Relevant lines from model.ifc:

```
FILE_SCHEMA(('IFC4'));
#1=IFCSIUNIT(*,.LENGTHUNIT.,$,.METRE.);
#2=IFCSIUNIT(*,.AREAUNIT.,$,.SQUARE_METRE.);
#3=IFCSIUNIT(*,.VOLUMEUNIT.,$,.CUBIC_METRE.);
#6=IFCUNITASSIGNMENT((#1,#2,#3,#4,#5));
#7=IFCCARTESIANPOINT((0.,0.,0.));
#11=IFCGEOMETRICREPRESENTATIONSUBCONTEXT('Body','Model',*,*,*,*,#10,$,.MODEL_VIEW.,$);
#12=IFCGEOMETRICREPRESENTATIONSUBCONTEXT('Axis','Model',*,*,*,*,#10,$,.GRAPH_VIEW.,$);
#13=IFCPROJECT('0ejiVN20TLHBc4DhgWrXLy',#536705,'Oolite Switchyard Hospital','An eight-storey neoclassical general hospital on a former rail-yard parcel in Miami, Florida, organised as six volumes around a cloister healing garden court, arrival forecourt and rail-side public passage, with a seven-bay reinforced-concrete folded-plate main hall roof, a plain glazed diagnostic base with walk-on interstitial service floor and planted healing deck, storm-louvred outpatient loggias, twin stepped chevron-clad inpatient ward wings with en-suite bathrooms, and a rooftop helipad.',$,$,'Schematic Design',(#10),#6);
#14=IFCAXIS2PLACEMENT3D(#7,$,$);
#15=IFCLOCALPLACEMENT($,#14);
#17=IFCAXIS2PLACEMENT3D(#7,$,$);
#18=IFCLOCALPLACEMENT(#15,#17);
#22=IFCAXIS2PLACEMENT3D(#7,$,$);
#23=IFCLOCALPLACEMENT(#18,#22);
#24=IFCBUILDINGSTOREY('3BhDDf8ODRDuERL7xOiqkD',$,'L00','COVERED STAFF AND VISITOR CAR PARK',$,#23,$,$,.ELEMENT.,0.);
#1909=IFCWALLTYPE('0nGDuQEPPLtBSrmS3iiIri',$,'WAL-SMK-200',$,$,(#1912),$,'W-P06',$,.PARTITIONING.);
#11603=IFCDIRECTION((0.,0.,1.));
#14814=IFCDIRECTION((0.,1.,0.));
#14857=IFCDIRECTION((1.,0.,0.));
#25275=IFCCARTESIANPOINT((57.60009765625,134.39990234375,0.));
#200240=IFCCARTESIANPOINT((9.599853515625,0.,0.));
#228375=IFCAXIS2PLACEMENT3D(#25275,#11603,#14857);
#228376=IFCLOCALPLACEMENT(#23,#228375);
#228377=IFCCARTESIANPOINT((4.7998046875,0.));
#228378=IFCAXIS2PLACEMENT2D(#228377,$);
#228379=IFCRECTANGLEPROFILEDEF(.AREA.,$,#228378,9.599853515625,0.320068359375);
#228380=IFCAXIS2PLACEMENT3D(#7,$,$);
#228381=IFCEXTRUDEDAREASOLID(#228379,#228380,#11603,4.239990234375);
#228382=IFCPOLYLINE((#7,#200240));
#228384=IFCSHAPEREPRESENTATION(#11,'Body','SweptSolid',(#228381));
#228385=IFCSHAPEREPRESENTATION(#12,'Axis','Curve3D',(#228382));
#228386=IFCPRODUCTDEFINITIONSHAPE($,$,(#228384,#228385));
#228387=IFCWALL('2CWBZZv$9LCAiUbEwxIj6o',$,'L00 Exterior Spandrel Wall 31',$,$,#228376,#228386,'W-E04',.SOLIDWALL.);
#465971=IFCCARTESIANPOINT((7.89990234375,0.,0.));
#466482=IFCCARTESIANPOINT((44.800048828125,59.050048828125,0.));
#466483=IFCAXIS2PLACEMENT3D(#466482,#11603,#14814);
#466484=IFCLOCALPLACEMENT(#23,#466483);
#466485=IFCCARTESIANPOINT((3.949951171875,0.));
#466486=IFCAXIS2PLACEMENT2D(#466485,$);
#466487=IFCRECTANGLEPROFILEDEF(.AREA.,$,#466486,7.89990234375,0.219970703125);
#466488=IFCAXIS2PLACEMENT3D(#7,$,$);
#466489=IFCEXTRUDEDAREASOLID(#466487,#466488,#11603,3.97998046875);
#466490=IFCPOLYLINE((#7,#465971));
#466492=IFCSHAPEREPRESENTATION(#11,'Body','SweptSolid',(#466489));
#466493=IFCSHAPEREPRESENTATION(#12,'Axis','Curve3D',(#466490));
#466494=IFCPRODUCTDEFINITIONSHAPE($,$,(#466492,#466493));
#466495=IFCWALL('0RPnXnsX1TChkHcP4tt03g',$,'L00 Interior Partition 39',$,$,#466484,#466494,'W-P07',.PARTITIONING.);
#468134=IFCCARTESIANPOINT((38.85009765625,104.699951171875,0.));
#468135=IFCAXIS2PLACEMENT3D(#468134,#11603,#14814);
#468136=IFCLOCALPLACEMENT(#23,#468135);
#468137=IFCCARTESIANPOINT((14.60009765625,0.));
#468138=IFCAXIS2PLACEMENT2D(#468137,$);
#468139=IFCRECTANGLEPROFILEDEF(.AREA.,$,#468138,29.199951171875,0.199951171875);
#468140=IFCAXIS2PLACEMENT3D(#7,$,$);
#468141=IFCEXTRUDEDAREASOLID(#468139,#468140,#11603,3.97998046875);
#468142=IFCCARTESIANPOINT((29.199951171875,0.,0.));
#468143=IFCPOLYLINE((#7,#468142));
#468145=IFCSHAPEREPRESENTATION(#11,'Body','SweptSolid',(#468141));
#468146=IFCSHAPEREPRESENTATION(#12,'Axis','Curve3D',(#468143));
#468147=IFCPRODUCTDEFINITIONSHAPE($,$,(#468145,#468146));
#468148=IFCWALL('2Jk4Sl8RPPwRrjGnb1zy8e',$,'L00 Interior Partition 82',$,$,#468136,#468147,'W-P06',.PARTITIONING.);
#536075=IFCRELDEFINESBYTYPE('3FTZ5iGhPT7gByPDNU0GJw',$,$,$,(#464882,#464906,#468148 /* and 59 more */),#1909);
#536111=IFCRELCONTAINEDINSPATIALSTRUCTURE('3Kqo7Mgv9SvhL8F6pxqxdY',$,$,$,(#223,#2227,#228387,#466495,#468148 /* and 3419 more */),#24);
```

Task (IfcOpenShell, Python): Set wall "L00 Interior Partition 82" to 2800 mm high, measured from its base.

```python
import ifcopenshell
import ifcopenshell.geom
import ifcopenshell.util.representation
import ifcopenshell.util.shape
import ifcopenshell.util.unit

model = ifcopenshell.open("model.ifc")
unit_scale = ifcopenshell.util.unit.calculate_unit_scale(model)
settings = ifcopenshell.geom.settings()


def volume(element):
    """Net volume in cubic metres, openings subtracted."""
    shape = ifcopenshell.geom.create_shape(settings, element)
    return ifcopenshell.util.shape.get_volume(shape.geometry)


wall = model.by_guid("2Jk4Sl8RPPwRrjGnb1zy8e")
before = volume(wall)

body = ifcopenshell.util.representation.get_representation(wall, "Model", "Body")
solid = body.Items[0]
old_height = solid.Depth
solid.Depth = 2.8 / unit_scale
after = volume(wall)

print(f"height {old_height:g} -> {solid.Depth:g}, volume {before:.3f} -> {after:.3f} m3")

model.write("model-out.ifc")
```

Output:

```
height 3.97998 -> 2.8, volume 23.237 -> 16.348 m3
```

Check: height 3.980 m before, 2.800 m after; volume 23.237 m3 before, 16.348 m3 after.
